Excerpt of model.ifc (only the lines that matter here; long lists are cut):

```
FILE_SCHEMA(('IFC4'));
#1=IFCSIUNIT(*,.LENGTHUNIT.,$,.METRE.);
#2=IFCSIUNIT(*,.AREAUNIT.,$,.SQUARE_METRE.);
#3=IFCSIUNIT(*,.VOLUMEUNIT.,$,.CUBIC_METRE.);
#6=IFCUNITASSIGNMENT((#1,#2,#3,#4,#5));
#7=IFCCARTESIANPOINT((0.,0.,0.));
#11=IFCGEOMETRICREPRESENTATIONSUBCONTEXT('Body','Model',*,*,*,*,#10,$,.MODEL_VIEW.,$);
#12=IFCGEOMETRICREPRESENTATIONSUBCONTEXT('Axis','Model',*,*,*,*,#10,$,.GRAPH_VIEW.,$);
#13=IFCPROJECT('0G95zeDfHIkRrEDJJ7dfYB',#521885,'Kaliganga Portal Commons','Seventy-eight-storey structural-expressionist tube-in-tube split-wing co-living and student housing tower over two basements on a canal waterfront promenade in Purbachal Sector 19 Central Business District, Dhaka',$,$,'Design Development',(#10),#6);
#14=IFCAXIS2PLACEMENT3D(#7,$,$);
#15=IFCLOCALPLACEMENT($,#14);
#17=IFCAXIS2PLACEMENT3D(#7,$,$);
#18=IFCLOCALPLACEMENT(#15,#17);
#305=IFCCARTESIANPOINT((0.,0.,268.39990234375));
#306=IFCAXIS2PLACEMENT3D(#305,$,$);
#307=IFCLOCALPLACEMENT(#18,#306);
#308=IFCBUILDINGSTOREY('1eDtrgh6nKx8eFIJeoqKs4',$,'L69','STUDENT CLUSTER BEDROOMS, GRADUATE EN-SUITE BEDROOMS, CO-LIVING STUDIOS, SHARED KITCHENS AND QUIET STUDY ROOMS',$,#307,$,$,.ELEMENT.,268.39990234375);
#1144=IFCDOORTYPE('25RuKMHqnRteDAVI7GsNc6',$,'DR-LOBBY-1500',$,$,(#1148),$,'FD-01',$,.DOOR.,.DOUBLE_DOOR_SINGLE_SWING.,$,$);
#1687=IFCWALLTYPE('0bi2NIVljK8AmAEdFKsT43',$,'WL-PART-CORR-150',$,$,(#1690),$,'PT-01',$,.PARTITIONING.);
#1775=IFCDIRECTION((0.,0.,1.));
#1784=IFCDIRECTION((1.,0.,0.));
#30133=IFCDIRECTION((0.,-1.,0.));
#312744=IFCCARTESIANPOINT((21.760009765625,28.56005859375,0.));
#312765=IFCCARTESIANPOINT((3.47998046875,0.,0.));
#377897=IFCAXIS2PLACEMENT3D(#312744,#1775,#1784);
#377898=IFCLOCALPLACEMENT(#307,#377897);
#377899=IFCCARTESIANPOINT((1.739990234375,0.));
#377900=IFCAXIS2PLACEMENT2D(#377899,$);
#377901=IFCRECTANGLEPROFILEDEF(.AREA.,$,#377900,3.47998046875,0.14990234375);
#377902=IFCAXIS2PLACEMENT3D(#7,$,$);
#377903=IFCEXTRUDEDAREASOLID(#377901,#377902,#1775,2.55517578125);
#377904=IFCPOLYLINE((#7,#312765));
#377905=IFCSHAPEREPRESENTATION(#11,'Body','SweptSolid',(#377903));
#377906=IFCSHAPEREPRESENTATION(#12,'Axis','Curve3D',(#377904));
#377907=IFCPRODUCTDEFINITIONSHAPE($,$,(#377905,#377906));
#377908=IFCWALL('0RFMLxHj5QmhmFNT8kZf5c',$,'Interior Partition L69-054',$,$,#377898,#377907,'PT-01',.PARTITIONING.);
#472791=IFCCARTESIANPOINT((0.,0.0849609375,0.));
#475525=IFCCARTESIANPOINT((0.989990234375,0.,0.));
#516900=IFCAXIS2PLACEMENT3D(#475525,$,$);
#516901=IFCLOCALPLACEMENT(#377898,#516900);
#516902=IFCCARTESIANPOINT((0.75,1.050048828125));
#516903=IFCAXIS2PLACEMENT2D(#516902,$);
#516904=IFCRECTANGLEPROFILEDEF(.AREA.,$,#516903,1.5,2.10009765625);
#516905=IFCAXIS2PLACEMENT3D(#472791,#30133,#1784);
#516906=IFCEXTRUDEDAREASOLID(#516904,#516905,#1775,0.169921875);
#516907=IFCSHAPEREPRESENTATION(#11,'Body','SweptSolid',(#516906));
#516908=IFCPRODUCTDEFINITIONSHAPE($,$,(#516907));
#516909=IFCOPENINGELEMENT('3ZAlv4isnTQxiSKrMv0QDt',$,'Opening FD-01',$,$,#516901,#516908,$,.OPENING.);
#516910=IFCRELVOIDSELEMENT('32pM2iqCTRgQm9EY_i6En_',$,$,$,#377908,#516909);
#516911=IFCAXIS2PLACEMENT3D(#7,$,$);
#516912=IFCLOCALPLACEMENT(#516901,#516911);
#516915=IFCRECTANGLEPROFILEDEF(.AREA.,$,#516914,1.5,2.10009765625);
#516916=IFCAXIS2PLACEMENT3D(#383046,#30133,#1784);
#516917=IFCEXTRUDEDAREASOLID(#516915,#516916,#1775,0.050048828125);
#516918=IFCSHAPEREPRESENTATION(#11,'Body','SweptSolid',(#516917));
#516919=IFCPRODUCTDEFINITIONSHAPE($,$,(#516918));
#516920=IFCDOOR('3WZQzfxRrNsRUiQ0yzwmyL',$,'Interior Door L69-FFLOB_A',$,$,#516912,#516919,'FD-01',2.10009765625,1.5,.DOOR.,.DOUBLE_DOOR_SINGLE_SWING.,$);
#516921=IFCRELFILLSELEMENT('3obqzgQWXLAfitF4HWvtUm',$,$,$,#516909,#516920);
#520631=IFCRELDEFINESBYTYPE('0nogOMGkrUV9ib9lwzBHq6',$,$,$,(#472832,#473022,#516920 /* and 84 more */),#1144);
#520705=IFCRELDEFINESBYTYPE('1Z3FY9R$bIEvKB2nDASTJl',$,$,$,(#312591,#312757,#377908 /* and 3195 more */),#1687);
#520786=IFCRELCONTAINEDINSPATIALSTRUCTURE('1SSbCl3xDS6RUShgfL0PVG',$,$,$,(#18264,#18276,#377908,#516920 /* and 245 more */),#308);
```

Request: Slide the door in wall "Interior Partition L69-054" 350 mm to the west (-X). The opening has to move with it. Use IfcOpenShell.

```python
import ifcopenshell
import ifcopenshell.api.geometry
import ifcopenshell.util.placement

model = ifcopenshell.open("model.ifc")

door = model.by_guid("3WZQzfxRrNsRUiQ0yzwmyL")
opening = door.FillsVoids[0].RelatingOpeningElement
wall = opening.VoidsElements[0].RelatingBuildingElement

wall_matrix = ifcopenshell.util.placement.get_local_placement(wall.ObjectPlacement)
shift = wall_matrix[:3, 0] * -0.35
before = ifcopenshell.util.placement.get_local_placement(door.ObjectPlacement)[:3, 3].copy()

# The door is placed relative to its opening, so it follows when the opening moves.
matrix = ifcopenshell.util.placement.get_local_placement(opening.ObjectPlacement)
matrix[:3, 3] += shift
ifcopenshell.api.geometry.edit_object_placement(
    model, product=opening, matrix=matrix, is_si=False, should_transform_children=True
)

after = ifcopenshell.util.placement.get_local_placement(door.ObjectPlacement)[:3, 3]
print("door moved by", (after - before).round(3) + 0.0)

model.write("model_edited.ifc")
```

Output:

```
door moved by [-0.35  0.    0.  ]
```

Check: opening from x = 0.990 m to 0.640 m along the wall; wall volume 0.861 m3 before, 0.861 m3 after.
